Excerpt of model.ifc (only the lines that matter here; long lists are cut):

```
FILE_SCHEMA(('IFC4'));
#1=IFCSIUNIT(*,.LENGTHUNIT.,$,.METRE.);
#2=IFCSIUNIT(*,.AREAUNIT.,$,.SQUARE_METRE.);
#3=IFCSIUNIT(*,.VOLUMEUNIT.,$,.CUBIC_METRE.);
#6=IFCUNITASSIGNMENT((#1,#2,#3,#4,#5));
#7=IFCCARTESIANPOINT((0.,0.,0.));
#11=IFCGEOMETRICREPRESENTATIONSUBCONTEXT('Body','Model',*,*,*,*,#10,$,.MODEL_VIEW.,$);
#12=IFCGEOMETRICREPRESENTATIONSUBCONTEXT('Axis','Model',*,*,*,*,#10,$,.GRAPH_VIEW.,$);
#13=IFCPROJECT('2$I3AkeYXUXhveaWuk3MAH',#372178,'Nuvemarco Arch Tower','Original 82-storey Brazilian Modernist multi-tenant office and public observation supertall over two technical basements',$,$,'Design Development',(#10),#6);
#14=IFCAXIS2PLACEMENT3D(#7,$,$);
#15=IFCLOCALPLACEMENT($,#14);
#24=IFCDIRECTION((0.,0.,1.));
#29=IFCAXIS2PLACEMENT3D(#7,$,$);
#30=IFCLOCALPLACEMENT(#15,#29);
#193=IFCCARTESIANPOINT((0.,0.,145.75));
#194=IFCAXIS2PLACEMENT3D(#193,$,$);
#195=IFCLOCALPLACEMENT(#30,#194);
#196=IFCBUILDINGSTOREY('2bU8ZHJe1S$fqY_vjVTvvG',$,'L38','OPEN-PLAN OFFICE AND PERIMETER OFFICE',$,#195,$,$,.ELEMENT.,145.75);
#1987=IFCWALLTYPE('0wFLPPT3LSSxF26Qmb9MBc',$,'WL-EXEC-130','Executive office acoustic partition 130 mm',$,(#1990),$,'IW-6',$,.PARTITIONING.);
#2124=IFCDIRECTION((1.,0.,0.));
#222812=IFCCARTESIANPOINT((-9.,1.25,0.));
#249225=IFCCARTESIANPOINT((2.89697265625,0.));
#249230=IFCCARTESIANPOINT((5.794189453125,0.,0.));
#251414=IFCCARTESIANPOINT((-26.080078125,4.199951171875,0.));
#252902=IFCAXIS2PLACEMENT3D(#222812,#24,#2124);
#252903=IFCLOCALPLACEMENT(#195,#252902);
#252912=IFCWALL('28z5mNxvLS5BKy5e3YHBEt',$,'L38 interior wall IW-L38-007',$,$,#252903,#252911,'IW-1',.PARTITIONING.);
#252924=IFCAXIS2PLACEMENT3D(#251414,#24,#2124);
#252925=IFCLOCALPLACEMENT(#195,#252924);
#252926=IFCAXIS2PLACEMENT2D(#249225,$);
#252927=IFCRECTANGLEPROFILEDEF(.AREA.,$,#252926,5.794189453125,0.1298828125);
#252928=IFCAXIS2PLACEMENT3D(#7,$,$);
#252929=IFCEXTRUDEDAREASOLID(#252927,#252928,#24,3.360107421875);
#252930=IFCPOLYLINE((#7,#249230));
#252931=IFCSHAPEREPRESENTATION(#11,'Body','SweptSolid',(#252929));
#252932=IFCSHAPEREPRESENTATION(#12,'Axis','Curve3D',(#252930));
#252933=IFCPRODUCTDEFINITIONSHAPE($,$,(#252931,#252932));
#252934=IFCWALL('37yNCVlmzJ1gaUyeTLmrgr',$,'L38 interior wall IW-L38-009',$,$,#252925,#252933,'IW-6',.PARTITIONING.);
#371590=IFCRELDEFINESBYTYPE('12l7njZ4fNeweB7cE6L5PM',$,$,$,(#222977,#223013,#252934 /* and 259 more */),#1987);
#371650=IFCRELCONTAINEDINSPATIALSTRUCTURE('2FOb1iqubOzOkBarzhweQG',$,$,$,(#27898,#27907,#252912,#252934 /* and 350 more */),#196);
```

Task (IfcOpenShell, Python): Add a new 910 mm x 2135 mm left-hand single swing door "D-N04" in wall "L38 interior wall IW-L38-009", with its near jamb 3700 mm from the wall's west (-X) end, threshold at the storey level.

```python
import numpy as np
import ifcopenshell
import ifcopenshell.api.feature
import ifcopenshell.api.geometry
import ifcopenshell.api.root
import ifcopenshell.api.spatial
import ifcopenshell.geom
import ifcopenshell.util.element
import ifcopenshell.util.placement
import ifcopenshell.util.representation
import ifcopenshell.util.shape
import ifcopenshell.util.unit

model = ifcopenshell.open("model.ifc")
unit_scale = ifcopenshell.util.unit.calculate_unit_scale(model)
settings = ifcopenshell.geom.settings()


def volume(element):
    """Net volume in cubic metres, openings subtracted."""
    shape = ifcopenshell.geom.create_shape(settings, element)
    return ifcopenshell.util.shape.get_volume(shape.geometry)


wall = model.by_guid("37yNCVlmzJ1gaUyeTLmrgr")
storey = ifcopenshell.util.element.get_container(wall, ifc_class="IfcBuildingStorey")
context = ifcopenshell.util.representation.get_context(model, "Model", "Body", "MODEL_VIEW")
before = volume(wall)

width, height, from_end, sill = 0.91, 2.135, 3.7, 0.0  # metres

# The wall runs along its own X axis, and the end named is its -X end.
wall_shape = ifcopenshell.geom.create_shape(settings, wall)
x, y, z = ifcopenshell.util.shape.get_vertices(wall_shape.geometry).T
start = x.min() + from_end
face, thickness = float(y.min()), float(y.max() - y.min())
wall_matrix = ifcopenshell.util.placement.get_local_placement(wall.ObjectPlacement)
level = ifcopenshell.util.placement.get_local_placement(storey.ObjectPlacement)[2, 3]


def in_wall(x, y):
    """Placement at x, y metres in the wall's axes, at sill height."""
    matrix = wall_matrix.copy()
    matrix[:, 3] = wall_matrix @ np.array([x / unit_scale, y / unit_scale, 0.0, 1.0])
    matrix[2, 3] = level + sill / unit_scale
    return matrix


# Opening: a box that overshoots both wall faces by 50 mm.
opening = ifcopenshell.api.root.create_entity(model, ifc_class="IfcOpeningElement", predefined_type="OPENING")
box = ifcopenshell.api.geometry.add_wall_representation(
    model, context=context, length=width, height=height, thickness=thickness + 0.1
)
ifcopenshell.api.geometry.assign_representation(model, product=opening, representation=box)
ifcopenshell.api.geometry.edit_object_placement(model, product=opening, matrix=in_wall(start, face - 0.05), is_si=False)
ifcopenshell.api.feature.add_feature(model, feature=opening, element=wall)

door = ifcopenshell.api.root.create_entity(model, ifc_class="IfcDoor", name="D-N04", predefined_type="DOOR")
door.OverallWidth, door.OverallHeight = width / unit_scale, height / unit_scale
door.OperationType = "SINGLE_SWING_LEFT"
body = ifcopenshell.api.geometry.add_door_representation(
    model,
    context=context,
    overall_width=door.OverallWidth,
    overall_height=door.OverallHeight,
    operation_type="SINGLE_SWING_LEFT",
    lining_properties={"LiningDepth": thickness / unit_scale, "ThresholdDepth": thickness / unit_scale},
)
ifcopenshell.api.geometry.assign_representation(model, product=door, representation=body)
ifcopenshell.api.spatial.assign_container(model, products=[door], relating_structure=storey)
ifcopenshell.api.feature.add_filling(model, opening=opening, element=door)

# The lining spans the wall, so the door starts at the wall face.
ifcopenshell.api.geometry.edit_object_placement(model, product=door, matrix=in_wall(start, face), is_si=False)

after = volume(wall)

print(f"wall volume {before:.3f} -> {after:.3f} m3")

model.write("model_edited.ifc")
```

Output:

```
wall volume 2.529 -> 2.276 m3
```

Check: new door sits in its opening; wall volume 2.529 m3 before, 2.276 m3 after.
